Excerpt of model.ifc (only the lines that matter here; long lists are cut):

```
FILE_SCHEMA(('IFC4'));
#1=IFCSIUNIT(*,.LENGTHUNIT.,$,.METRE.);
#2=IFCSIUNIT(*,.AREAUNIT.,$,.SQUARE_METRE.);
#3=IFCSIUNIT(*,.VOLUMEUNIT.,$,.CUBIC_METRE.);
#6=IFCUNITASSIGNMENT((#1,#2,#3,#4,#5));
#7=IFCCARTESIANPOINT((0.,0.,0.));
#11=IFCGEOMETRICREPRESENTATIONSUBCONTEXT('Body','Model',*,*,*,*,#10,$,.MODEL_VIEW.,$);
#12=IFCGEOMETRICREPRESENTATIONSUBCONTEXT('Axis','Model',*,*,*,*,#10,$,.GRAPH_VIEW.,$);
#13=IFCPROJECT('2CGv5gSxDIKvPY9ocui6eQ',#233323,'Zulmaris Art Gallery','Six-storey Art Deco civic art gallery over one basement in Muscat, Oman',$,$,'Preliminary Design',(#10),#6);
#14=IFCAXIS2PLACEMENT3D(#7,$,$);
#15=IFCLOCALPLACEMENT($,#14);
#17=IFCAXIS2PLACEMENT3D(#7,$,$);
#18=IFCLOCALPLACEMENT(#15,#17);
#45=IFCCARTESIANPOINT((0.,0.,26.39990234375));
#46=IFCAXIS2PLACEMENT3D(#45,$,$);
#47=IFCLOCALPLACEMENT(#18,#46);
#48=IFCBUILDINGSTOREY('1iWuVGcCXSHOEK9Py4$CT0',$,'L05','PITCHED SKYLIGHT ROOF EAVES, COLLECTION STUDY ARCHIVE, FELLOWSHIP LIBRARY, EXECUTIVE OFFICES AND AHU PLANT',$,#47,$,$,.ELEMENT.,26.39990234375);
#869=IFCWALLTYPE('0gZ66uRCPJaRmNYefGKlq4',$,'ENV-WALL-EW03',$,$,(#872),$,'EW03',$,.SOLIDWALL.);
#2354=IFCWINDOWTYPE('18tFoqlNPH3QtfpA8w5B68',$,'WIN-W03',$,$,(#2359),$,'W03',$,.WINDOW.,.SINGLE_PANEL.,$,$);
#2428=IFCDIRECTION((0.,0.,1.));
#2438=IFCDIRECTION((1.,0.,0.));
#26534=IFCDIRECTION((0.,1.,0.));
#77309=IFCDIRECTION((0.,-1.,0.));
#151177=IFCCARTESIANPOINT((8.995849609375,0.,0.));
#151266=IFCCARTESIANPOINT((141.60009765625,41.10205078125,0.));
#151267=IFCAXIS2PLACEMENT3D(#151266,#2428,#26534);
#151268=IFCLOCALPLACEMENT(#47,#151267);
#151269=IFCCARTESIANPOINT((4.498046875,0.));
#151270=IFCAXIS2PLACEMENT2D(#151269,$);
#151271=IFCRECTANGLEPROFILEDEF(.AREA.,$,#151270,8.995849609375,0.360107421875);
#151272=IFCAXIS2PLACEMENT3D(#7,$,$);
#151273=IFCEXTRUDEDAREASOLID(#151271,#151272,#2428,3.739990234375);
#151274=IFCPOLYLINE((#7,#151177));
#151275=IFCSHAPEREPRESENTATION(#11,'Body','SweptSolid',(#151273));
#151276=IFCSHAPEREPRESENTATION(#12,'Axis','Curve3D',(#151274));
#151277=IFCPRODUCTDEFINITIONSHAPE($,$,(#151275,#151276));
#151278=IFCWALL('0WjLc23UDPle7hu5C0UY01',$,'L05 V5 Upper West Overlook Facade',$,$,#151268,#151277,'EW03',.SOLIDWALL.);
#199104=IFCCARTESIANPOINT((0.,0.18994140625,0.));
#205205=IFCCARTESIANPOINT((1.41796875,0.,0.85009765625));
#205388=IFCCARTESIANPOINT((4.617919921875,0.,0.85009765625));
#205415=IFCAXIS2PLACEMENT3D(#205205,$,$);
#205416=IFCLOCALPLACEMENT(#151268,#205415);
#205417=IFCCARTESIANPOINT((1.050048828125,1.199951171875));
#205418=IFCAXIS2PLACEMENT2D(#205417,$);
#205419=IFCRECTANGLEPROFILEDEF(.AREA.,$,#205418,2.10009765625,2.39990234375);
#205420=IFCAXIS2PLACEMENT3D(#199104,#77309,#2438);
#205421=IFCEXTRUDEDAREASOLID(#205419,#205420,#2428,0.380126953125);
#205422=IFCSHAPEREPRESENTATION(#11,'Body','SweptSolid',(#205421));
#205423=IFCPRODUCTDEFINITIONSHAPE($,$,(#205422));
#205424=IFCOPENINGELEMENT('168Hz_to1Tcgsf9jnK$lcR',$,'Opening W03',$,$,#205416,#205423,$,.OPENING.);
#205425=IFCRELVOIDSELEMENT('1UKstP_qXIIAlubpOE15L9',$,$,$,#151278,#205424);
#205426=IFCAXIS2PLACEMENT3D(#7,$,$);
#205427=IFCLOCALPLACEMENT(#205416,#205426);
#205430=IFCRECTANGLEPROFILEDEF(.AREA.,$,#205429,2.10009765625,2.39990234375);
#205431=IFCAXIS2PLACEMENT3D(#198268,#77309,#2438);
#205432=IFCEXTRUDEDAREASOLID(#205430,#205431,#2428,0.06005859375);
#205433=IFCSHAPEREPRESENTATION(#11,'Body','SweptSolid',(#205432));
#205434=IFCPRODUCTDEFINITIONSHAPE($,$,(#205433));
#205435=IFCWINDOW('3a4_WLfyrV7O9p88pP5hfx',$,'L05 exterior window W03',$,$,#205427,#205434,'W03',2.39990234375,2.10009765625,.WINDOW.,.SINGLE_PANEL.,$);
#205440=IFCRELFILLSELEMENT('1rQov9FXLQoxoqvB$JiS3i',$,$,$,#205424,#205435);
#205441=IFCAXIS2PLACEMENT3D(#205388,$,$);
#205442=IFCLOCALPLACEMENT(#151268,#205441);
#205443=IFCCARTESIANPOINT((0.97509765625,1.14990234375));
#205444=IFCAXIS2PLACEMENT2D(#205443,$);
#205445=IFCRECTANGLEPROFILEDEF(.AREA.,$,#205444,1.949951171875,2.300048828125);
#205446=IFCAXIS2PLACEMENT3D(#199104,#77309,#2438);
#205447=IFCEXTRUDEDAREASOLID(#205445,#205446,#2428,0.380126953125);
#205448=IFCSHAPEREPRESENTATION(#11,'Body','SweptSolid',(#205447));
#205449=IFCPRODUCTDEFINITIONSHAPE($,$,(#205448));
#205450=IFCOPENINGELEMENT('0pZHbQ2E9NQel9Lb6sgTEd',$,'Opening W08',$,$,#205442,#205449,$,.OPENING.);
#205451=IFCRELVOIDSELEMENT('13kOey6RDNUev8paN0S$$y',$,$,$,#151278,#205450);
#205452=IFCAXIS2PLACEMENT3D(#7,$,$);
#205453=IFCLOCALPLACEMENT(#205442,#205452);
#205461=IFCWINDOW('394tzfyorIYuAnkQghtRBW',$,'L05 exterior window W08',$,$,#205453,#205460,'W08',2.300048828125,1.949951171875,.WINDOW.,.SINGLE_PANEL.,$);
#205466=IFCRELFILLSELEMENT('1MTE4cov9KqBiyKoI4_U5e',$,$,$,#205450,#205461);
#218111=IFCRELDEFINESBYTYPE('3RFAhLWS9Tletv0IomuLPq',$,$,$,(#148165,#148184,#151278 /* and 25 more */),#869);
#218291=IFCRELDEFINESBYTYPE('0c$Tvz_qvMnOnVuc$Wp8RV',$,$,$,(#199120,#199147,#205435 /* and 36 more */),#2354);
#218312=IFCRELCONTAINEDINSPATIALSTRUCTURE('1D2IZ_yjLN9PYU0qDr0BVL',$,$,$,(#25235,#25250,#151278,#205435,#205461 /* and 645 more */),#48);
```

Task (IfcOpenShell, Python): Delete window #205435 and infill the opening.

```python
import ifcopenshell
import ifcopenshell.api.feature
import ifcopenshell.api.root
import ifcopenshell.geom
import ifcopenshell.util.shape

model = ifcopenshell.open("model.ifc")
settings = ifcopenshell.geom.settings()


def volume(element):
    """Net volume in cubic metres, openings subtracted."""
    shape = ifcopenshell.geom.create_shape(settings, element)
    return ifcopenshell.util.shape.get_volume(shape.geometry)


window = model.by_guid("3a4_WLfyrV7O9p88pP5hfx")
opening = window.FillsVoids[0].RelatingOpeningElement
wall = opening.VoidsElements[0].RelatingBuildingElement
before = volume(wall)

ifcopenshell.api.root.remove_product(model, product=window)
ifcopenshell.api.feature.remove_feature(model, feature=opening)

after = volume(wall)

print(f"wall volume {before:.3f} -> {after:.3f} m3")

model.write("model_edited.ifc")
```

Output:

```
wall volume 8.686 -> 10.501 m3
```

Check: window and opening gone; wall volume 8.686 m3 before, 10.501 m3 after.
